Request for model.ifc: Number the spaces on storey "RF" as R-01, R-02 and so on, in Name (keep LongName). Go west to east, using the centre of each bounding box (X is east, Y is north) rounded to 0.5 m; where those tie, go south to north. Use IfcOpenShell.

First a look at what the model holds.

```python
import ifcopenshell
import ifcopenshell.util.element
import ifcopenshell.util.placement

model = ifcopenshell.open("model.ifc")
print(model.schema)
storey = next(s for s in model.by_type("IfcBuildingStorey") if s.Name == "RF")
spaces = [e for e in ifcopenshell.util.element.get_decomposition(storey) if e.is_a("IfcSpace")]
for e in sorted(spaces, key=lambda e: e.id()):
    origin = ifcopenshell.util.placement.get_local_placement(e.ObjectPlacement)[:3, 3]
    print(e.id(), e.Name, e.LongName, origin.round(2) + 0.0, sep=" | ")
```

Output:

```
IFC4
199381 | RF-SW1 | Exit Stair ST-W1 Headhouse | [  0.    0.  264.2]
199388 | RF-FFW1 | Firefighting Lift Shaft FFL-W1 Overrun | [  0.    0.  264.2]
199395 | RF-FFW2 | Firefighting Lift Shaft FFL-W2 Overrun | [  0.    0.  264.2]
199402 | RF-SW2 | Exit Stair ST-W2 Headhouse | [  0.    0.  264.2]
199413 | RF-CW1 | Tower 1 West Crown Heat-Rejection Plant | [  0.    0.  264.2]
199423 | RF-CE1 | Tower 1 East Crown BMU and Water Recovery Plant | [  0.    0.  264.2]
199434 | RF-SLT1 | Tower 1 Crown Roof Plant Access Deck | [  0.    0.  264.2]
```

```python
import ifcopenshell
import ifcopenshell.geom
import ifcopenshell.util.element
import ifcopenshell.util.shape

model = ifcopenshell.open("model.ifc")
settings = ifcopenshell.geom.settings()
settings.set("use-world-coords", True)


def centre(element):
    shape = ifcopenshell.geom.create_shape(settings, element)
    return ifcopenshell.util.shape.get_bbox_centroid(shape.geometry)


storey = next(s for s in model.by_type("IfcBuildingStorey") if s.Name == "RF")
spaces = [e for e in ifcopenshell.util.element.get_decomposition(storey) if e.is_a("IfcSpace")]

# Insertion points can sit at a corner or the storey origin, so sort by the geometry (in metres).
centres = {e: centre(e) for e in spaces}
spaces.sort(key=lambda e: (round(centres[e][0] / 0.5), centres[e][1]))

for i, e in enumerate(spaces, start=1):
    number = f"R-{i:02d}"
    e.Name = number
    print(e.id(), number)

model.write("model_v2.ifc")
```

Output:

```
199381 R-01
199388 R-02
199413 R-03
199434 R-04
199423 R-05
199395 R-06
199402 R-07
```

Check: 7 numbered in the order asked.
